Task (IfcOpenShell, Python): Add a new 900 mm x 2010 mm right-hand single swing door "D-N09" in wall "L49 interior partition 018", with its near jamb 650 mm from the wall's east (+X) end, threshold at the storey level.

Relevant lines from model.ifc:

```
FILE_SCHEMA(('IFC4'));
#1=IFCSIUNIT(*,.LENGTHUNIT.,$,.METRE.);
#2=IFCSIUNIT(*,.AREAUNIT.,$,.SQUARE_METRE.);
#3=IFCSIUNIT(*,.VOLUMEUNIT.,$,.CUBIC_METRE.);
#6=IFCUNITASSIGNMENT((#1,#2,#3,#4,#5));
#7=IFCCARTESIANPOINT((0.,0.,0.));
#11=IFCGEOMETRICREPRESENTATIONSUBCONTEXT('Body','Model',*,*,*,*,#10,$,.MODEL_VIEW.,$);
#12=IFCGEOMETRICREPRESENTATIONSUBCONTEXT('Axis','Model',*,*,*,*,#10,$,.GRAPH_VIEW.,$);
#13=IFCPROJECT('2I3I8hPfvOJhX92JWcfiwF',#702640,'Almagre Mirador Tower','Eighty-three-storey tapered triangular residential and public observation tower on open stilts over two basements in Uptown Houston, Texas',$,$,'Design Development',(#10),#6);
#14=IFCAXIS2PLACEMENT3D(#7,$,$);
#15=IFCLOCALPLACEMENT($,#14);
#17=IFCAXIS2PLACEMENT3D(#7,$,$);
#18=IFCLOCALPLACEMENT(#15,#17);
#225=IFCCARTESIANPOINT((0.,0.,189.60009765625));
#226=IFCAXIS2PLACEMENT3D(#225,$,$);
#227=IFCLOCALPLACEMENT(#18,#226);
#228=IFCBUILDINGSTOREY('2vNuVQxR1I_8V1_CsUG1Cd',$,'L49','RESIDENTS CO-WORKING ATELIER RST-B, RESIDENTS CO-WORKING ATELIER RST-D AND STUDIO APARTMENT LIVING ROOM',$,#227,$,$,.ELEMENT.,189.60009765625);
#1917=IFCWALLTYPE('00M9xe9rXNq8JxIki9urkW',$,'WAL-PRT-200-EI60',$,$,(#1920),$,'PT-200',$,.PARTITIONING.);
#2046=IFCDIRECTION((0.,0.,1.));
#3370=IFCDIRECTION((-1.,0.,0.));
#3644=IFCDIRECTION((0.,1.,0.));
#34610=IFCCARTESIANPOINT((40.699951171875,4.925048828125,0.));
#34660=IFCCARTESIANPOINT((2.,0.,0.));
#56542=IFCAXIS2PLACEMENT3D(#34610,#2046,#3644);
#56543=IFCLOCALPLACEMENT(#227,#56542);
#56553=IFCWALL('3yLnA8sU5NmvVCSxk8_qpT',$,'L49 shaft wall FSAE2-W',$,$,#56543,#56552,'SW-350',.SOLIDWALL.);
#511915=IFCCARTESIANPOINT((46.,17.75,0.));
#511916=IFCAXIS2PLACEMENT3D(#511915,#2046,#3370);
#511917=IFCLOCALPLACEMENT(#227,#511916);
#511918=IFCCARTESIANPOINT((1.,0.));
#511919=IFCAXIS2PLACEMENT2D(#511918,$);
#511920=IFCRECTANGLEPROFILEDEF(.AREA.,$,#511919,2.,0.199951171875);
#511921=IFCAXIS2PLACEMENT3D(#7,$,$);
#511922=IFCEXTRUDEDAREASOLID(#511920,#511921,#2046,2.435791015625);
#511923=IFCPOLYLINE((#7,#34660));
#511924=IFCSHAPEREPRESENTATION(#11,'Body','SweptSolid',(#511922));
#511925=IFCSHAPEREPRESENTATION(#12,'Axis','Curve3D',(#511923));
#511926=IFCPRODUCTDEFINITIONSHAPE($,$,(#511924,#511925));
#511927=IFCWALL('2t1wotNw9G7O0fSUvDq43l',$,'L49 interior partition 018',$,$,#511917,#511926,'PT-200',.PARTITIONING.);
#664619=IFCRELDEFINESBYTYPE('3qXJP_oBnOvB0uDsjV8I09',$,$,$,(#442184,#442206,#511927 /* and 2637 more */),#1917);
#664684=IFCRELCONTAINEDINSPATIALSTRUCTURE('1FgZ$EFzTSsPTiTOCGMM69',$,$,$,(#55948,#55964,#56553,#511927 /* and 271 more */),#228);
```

```python
import numpy as np
import ifcopenshell
import ifcopenshell.api.feature
import ifcopenshell.api.geometry
import ifcopenshell.api.root
import ifcopenshell.api.spatial
import ifcopenshell.geom
import ifcopenshell.util.element
import ifcopenshell.util.placement
import ifcopenshell.util.representation
import ifcopenshell.util.shape
import ifcopenshell.util.unit

model = ifcopenshell.open("model.ifc")
unit_scale = ifcopenshell.util.unit.calculate_unit_scale(model)
settings = ifcopenshell.geom.settings()


def volume(element):
    """Net volume in cubic metres, openings subtracted."""
    shape = ifcopenshell.geom.create_shape(settings, element)
    return ifcopenshell.util.shape.get_volume(shape.geometry)


wall = model.by_guid("2t1wotNw9G7O0fSUvDq43l")
storey = ifcopenshell.util.element.get_container(wall, ifc_class="IfcBuildingStorey")
context = ifcopenshell.util.representation.get_context(model, "Model", "Body", "MODEL_VIEW")
before = volume(wall)

width, height, from_end, sill = 0.9, 2.01, 0.65, 0.0  # metres

# The wall runs along its own X axis, and the end named is its -X end.
wall_shape = ifcopenshell.geom.create_shape(settings, wall)
x, y, z = ifcopenshell.util.shape.get_vertices(wall_shape.geometry).T
start = x.min() + from_end
face, thickness = float(y.min()), float(y.max() - y.min())
wall_matrix = ifcopenshell.util.placement.get_local_placement(wall.ObjectPlacement)
level = ifcopenshell.util.placement.get_local_placement(storey.ObjectPlacement)[2, 3]


def in_wall(x, y):
    """Placement at x, y metres in the wall's axes, at sill height."""
    matrix = wall_matrix.copy()
    matrix[:, 3] = wall_matrix @ np.array([x / unit_scale, y / unit_scale, 0.0, 1.0])
    matrix[2, 3] = level + sill / unit_scale
    return matrix


# Opening: a box that overshoots both wall faces by 50 mm.
opening = ifcopenshell.api.root.create_entity(model, ifc_class="IfcOpeningElement", predefined_type="OPENING")
box = ifcopenshell.api.geometry.add_wall_representation(
    model, context=context, length=width, height=height, thickness=thickness + 0.1
)
ifcopenshell.api.geometry.assign_representation(model, product=opening, representation=box)
ifcopenshell.api.geometry.edit_object_placement(model, product=opening, matrix=in_wall(start, face - 0.05), is_si=False)
ifcopenshell.api.feature.add_feature(model, feature=opening, element=wall)

door = ifcopenshell.api.root.create_entity(model, ifc_class="IfcDoor", name="D-N09", predefined_type="DOOR")
door.OverallWidth, door.OverallHeight = width / unit_scale, height / unit_scale
door.OperationType = "SINGLE_SWING_RIGHT"
body = ifcopenshell.api.geometry.add_door_representation(
    model,
    context=context,
    overall_width=door.OverallWidth,
    overall_height=door.OverallHeight,
    operation_type="SINGLE_SWING_RIGHT",
    lining_properties={"LiningDepth": thickness / unit_scale, "ThresholdDepth": thickness / unit_scale},
)
ifcopenshell.api.geometry.assign_representation(model, product=door, representation=body)
ifcopenshell.api.spatial.assign_container(model, products=[door], relating_structure=storey)
ifcopenshell.api.feature.add_filling(model, opening=opening, element=door)

# The lining spans the wall, so the door starts at the wall face.
ifcopenshell.api.geometry.edit_object_placement(model, product=door, matrix=in_wall(start, face), is_si=False)

after = volume(wall)

print(f"wall volume {before:.3f} -> {after:.3f} m3")

model.write("model_v2.ifc")
```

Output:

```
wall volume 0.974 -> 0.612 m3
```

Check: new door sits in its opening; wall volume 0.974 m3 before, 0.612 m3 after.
